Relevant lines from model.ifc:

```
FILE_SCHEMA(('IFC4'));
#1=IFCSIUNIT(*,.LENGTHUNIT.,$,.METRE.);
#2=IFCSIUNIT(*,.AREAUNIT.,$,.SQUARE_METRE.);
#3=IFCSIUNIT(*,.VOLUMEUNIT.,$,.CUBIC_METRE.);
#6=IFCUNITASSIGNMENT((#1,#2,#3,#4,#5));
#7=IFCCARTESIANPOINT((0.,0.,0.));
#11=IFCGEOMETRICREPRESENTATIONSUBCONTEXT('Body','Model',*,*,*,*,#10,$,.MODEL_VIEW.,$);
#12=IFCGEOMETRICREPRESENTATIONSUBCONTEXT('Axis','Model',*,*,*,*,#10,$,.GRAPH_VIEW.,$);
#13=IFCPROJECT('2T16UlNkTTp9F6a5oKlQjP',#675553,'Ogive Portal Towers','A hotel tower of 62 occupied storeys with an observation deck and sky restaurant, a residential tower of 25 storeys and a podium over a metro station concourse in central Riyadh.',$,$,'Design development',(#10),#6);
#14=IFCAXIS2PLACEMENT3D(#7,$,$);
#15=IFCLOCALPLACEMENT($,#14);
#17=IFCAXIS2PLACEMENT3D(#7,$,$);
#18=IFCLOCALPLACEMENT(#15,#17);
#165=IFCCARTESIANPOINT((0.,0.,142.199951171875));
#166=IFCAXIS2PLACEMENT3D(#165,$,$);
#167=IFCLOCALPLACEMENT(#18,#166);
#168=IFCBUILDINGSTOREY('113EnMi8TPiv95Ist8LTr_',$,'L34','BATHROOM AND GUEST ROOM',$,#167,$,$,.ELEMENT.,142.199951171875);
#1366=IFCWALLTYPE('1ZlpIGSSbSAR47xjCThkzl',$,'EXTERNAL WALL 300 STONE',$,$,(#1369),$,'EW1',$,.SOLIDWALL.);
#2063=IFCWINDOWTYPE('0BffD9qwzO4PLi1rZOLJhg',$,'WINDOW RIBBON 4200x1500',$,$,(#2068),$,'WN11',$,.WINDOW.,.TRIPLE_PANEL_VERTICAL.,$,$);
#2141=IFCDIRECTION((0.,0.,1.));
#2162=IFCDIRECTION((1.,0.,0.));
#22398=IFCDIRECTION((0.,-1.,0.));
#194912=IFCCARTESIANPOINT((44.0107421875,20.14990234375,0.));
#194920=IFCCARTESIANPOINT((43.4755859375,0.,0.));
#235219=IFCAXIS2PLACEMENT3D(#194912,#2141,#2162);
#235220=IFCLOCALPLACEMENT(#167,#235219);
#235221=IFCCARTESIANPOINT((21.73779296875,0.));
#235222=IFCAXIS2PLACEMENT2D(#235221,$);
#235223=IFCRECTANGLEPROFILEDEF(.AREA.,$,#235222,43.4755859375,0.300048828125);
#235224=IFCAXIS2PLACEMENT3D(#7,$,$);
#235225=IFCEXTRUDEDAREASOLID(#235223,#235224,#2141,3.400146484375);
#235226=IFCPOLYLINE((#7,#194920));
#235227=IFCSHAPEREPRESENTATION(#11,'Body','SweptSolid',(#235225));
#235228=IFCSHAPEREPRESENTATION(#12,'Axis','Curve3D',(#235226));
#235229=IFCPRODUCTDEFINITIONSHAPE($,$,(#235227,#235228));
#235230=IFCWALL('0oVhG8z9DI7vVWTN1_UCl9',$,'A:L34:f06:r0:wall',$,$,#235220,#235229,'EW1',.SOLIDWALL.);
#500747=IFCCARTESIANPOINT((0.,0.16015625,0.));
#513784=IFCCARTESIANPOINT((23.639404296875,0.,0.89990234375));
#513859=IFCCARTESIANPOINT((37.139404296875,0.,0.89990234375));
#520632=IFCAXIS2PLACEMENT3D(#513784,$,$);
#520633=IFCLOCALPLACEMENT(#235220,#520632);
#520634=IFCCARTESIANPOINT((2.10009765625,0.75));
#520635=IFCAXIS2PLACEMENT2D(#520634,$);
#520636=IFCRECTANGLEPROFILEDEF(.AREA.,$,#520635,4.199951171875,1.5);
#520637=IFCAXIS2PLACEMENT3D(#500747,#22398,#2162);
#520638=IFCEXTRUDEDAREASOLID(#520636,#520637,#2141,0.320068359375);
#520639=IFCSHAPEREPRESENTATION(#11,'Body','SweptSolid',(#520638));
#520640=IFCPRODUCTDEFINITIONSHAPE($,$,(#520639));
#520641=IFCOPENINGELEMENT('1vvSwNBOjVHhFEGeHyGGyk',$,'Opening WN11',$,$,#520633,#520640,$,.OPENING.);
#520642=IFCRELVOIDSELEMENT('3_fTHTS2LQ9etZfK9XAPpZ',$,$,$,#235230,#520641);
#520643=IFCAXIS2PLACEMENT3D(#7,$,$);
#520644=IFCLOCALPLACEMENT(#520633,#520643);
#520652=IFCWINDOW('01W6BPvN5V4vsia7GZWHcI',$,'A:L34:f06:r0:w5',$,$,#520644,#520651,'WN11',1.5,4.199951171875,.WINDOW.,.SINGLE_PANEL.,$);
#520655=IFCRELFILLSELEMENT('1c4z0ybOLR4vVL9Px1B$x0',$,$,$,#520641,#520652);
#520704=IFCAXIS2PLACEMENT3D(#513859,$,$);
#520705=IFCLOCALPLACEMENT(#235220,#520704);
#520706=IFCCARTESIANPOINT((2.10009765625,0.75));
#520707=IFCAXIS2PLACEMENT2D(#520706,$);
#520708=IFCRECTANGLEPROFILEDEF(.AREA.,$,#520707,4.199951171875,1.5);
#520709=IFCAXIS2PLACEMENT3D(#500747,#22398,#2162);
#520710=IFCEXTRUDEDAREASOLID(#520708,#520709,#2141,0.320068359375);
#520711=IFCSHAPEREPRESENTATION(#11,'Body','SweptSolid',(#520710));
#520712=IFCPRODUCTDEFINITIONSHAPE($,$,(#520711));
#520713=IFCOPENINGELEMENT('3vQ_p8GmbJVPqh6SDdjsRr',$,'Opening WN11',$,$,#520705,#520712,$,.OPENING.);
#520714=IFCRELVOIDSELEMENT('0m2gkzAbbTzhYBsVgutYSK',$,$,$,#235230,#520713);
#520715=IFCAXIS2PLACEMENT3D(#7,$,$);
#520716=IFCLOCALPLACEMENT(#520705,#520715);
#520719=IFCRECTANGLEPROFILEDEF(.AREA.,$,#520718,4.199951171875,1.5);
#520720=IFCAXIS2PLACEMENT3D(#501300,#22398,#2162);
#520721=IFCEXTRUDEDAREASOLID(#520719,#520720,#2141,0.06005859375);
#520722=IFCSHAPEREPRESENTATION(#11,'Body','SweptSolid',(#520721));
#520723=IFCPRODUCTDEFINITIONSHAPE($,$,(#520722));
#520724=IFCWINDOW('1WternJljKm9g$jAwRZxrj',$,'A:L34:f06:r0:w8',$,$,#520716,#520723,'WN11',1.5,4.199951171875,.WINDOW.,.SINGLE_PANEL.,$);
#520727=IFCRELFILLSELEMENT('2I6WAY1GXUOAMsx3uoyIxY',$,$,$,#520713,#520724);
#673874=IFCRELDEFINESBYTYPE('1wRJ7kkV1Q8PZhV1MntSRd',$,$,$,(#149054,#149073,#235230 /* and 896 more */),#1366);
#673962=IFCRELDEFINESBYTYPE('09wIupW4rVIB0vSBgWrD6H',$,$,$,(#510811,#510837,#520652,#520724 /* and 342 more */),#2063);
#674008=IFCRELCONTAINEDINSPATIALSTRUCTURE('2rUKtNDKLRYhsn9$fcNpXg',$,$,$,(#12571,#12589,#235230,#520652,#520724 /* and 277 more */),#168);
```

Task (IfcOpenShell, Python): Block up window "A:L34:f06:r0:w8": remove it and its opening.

```python
import ifcopenshell
import ifcopenshell.api.feature
import ifcopenshell.api.root
import ifcopenshell.geom
import ifcopenshell.util.shape

model = ifcopenshell.open("model.ifc")
settings = ifcopenshell.geom.settings()


def volume(element):
    """Net volume in cubic metres, openings subtracted."""
    shape = ifcopenshell.geom.create_shape(settings, element)
    return ifcopenshell.util.shape.get_volume(shape.geometry)


window = model.by_id(520724)
opening = window.FillsVoids[0].RelatingOpeningElement
wall = opening.VoidsElements[0].RelatingBuildingElement
before = volume(wall)

ifcopenshell.api.root.remove_product(model, product=window)
ifcopenshell.api.feature.remove_feature(model, feature=opening)

after = volume(wall)

print(f"wall volume {before:.3f} -> {after:.3f} m3")

model.write("model_updated.ifc")
```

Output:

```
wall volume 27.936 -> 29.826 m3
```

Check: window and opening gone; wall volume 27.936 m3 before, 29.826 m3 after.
